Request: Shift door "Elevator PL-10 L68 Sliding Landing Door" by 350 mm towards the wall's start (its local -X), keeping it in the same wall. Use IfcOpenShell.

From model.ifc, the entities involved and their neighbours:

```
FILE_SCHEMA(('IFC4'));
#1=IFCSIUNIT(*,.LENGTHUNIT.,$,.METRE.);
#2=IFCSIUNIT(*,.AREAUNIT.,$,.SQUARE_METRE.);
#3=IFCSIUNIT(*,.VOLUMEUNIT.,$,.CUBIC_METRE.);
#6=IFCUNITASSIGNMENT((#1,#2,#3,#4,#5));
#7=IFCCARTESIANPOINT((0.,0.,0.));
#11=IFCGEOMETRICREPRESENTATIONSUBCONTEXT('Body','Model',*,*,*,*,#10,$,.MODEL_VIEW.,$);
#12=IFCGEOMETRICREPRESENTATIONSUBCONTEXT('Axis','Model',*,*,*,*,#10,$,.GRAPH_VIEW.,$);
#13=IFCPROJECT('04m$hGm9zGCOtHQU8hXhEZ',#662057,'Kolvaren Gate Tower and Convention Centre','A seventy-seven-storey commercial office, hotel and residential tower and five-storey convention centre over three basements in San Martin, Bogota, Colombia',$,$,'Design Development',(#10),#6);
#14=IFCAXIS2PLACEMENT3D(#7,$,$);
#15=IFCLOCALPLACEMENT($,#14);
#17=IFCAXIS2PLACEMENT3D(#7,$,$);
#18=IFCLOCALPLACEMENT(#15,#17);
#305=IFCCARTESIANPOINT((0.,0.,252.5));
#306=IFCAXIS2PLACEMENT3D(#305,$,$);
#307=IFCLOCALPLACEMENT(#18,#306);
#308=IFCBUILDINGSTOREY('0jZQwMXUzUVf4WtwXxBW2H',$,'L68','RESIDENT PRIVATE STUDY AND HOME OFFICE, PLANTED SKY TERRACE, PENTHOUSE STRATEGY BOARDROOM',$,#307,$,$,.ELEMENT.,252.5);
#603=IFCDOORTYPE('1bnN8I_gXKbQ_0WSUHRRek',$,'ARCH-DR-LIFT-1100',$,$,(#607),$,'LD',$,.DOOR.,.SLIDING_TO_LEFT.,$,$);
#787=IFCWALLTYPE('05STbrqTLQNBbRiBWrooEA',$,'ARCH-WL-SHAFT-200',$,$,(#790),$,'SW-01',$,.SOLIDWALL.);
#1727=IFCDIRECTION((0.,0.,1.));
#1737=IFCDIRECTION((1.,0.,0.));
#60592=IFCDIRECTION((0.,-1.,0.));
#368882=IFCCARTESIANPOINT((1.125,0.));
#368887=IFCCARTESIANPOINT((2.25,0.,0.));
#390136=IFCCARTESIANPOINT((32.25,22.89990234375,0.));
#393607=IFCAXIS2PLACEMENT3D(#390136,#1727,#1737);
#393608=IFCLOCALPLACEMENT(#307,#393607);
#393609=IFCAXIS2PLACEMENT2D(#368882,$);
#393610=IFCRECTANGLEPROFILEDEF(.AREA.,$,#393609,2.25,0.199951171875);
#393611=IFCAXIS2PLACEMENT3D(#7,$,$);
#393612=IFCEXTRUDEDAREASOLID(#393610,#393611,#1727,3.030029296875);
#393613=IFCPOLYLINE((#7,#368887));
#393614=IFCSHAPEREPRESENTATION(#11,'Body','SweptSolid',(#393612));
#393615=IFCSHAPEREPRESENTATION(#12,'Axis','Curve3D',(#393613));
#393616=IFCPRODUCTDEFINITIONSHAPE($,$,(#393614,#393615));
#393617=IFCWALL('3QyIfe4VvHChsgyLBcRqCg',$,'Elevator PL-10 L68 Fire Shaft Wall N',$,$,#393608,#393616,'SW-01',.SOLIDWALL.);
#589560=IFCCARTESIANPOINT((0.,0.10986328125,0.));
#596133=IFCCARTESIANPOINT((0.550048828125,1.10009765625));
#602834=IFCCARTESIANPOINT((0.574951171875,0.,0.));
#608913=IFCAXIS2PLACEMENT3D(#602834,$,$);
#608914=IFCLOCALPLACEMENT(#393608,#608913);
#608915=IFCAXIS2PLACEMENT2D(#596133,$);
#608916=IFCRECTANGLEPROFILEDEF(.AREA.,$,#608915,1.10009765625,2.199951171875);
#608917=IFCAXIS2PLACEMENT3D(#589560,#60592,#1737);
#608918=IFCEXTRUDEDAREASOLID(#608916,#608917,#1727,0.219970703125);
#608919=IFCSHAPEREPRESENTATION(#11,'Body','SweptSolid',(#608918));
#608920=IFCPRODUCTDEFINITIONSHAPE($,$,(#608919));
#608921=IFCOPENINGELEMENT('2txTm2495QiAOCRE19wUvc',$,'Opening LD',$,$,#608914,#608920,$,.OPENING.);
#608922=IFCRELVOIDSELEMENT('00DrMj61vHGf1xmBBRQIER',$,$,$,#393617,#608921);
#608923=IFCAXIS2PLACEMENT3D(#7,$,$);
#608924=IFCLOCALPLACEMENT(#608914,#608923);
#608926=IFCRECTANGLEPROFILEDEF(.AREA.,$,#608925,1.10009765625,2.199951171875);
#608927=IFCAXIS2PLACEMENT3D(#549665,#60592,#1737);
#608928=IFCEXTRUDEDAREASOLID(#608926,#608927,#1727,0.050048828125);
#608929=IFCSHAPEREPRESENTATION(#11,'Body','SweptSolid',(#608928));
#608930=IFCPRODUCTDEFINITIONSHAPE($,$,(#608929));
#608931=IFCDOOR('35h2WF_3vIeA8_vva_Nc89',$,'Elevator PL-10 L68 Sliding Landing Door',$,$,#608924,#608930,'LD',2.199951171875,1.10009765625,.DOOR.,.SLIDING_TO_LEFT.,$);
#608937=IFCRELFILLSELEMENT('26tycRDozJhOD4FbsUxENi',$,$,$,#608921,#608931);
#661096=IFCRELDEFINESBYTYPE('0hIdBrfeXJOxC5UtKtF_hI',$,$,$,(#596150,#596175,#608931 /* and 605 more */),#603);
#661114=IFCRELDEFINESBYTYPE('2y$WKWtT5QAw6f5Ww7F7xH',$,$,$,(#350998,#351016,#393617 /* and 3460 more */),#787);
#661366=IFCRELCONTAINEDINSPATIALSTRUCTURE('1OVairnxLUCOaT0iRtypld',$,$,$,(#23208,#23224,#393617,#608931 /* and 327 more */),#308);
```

```python
import ifcopenshell
import ifcopenshell.api.geometry
import ifcopenshell.util.placement
import ifcopenshell.util.unit

model = ifcopenshell.open("model.ifc")
unit_scale = ifcopenshell.util.unit.calculate_unit_scale(model)

door = model.by_id(608931)
opening = door.FillsVoids[0].RelatingOpeningElement
wall = opening.VoidsElements[0].RelatingBuildingElement

wall_matrix = ifcopenshell.util.placement.get_local_placement(wall.ObjectPlacement)
shift = wall_matrix[:3, 0] * -0.35 / unit_scale
before = ifcopenshell.util.placement.get_local_placement(door.ObjectPlacement)[:3, 3].copy()

# The door is placed relative to its opening, so it follows when the opening moves.
matrix = ifcopenshell.util.placement.get_local_placement(opening.ObjectPlacement)
matrix[:3, 3] += shift
ifcopenshell.api.geometry.edit_object_placement(
    model, product=opening, matrix=matrix, is_si=False, should_transform_children=True
)

after = ifcopenshell.util.placement.get_local_placement(door.ObjectPlacement)[:3, 3]
print("door moved by", (after - before).round(3) + 0.0)

model.write("model_edited.ifc")
```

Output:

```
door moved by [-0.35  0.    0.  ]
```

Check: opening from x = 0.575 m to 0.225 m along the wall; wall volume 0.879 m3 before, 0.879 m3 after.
